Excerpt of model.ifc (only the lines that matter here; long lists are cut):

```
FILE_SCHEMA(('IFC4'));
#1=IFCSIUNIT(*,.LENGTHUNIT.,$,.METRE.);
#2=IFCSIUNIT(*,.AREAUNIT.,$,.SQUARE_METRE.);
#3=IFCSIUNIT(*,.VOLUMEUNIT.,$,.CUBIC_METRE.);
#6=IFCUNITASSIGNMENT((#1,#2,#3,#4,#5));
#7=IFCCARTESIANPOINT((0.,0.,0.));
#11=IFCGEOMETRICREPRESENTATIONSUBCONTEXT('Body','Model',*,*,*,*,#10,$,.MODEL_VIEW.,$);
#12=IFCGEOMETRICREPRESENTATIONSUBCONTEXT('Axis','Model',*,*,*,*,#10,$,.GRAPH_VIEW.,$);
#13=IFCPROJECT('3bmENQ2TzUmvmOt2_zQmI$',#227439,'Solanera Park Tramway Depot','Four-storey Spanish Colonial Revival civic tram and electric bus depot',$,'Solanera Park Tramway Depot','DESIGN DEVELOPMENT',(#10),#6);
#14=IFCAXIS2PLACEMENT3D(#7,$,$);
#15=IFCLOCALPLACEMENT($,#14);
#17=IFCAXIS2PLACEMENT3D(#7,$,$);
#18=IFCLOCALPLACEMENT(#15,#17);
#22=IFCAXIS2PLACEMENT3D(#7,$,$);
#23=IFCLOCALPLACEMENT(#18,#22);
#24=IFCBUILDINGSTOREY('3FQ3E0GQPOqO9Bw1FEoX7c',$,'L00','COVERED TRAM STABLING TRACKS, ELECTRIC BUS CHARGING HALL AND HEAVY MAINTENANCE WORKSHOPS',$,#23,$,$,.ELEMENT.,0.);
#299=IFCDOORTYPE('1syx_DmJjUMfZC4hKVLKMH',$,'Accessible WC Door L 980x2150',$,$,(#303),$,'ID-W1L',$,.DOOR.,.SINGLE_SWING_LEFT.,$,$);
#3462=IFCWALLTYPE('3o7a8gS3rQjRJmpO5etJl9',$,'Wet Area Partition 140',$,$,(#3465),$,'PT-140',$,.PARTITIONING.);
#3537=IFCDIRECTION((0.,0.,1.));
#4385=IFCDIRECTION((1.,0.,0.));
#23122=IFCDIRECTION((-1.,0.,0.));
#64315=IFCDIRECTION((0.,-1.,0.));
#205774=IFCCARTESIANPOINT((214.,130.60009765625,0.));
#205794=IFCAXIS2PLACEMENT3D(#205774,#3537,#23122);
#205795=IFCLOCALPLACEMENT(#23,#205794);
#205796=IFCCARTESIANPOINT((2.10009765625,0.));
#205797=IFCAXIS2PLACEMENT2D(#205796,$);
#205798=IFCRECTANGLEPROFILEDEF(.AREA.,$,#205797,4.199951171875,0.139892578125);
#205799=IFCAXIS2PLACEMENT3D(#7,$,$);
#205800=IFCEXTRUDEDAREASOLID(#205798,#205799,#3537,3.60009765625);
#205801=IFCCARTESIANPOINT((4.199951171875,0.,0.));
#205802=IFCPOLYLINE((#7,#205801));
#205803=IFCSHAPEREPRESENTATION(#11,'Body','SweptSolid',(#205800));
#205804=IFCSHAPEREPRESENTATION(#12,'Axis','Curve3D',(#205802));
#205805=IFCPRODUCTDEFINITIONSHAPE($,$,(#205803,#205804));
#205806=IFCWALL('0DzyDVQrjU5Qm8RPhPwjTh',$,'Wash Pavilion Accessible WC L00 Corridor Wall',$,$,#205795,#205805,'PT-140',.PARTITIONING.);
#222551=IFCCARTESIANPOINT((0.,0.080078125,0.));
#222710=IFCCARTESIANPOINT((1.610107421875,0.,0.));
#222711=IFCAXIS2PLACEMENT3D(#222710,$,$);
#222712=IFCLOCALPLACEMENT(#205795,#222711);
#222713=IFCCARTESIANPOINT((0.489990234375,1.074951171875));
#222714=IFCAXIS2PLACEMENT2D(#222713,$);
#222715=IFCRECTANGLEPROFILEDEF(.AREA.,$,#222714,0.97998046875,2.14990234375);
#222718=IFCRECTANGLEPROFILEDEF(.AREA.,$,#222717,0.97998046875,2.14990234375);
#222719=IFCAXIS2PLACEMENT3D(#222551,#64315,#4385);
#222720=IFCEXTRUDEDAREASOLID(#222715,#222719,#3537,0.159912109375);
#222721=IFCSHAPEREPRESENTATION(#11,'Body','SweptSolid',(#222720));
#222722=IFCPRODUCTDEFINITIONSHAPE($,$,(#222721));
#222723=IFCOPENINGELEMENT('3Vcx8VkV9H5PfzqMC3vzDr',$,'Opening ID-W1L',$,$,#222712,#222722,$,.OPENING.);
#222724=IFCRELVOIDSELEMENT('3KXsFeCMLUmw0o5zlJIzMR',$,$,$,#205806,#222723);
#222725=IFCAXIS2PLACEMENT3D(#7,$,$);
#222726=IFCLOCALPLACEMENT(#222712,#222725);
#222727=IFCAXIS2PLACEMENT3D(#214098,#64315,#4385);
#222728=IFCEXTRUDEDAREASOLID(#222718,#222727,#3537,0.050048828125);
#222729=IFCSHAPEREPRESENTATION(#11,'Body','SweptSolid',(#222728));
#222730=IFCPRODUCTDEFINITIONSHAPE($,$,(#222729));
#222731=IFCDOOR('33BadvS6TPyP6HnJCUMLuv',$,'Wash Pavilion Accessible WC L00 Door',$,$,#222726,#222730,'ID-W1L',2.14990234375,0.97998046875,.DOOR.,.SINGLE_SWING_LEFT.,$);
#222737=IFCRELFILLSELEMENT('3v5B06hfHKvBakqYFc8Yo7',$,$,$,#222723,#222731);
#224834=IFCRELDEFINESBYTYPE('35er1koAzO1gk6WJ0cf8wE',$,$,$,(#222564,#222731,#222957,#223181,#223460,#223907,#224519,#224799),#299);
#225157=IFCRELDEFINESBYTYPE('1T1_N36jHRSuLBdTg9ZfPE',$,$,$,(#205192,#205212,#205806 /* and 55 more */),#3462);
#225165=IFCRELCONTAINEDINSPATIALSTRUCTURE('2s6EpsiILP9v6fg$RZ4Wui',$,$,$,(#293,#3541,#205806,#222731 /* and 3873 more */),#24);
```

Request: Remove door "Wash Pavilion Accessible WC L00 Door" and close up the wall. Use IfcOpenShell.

```python
import ifcopenshell
import ifcopenshell.api.feature
import ifcopenshell.api.root
import ifcopenshell.geom
import ifcopenshell.util.shape

model = ifcopenshell.open("model.ifc")
settings = ifcopenshell.geom.settings()


def volume(element):
    """Net volume in cubic metres, openings subtracted."""
    shape = ifcopenshell.geom.create_shape(settings, element)
    return ifcopenshell.util.shape.get_volume(shape.geometry)


door = model.by_guid("33BadvS6TPyP6HnJCUMLuv")
opening = door.FillsVoids[0].RelatingOpeningElement
wall = opening.VoidsElements[0].RelatingBuildingElement
before = volume(wall)

ifcopenshell.api.root.remove_product(model, product=door)
ifcopenshell.api.feature.remove_feature(model, feature=opening)

after = volume(wall)

print(f"wall volume {before:.3f} -> {after:.3f} m3")

model.write("model_edited.ifc")
```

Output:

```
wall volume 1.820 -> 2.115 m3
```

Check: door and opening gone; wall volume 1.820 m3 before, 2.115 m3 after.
